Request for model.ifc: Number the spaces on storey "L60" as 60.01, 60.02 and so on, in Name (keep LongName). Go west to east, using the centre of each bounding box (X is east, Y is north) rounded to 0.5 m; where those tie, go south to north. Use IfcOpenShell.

First a look at what the model holds.

```python
import ifcopenshell
import ifcopenshell.util.element
import ifcopenshell.util.placement

model = ifcopenshell.open("model.ifc")
print(model.schema)
storey = next(s for s in model.by_type("IfcBuildingStorey") if s.Name == "L60")
spaces = [e for e in ifcopenshell.util.element.get_decomposition(storey) if e.is_a("IfcSpace")]
for e in sorted(spaces, key=lambda e: e.id()):
    origin = ifcopenshell.util.placement.get_local_placement(e.ObjectPlacement)[:3, 3]
    print(e.id(), e.Name, e.LongName, origin.round(2) + 0.0, sep=" | ")
```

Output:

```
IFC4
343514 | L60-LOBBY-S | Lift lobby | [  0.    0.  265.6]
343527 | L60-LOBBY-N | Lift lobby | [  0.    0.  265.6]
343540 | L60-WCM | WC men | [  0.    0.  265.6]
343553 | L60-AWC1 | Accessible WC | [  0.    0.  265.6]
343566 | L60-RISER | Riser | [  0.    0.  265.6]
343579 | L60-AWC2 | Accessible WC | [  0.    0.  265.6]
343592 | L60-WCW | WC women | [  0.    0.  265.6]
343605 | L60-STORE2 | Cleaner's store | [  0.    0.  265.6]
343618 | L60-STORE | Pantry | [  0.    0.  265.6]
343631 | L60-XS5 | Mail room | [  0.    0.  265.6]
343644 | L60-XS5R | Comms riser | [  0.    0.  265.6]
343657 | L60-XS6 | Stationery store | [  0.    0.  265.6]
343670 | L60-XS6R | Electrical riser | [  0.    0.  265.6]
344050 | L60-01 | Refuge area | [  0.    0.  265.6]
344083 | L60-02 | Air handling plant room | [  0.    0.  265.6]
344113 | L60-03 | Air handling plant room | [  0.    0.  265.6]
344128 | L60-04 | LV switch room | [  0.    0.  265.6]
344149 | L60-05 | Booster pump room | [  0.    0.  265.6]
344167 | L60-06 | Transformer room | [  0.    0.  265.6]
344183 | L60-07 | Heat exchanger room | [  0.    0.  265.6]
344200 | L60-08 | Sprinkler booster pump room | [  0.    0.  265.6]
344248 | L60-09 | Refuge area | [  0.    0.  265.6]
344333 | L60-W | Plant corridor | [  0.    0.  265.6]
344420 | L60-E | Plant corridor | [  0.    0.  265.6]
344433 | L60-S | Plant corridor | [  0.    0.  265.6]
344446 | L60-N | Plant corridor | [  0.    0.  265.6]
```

```python
import ifcopenshell
import ifcopenshell.geom
import ifcopenshell.util.element
import ifcopenshell.util.shape

model = ifcopenshell.open("model.ifc")
settings = ifcopenshell.geom.settings()
settings.set("use-world-coords", True)


def centre(element):
    shape = ifcopenshell.geom.create_shape(settings, element)
    return ifcopenshell.util.shape.get_bbox_centroid(shape.geometry)


storey = next(s for s in model.by_type("IfcBuildingStorey") if s.Name == "L60")
spaces = [e for e in ifcopenshell.util.element.get_decomposition(storey) if e.is_a("IfcSpace")]

# Insertion points can sit at a corner or the storey origin, so sort by the geometry (in metres).
centres = {e: centre(e) for e in spaces}
spaces.sort(key=lambda e: (round(centres[e][0] / 0.5), centres[e][1]))

for i, e in enumerate(spaces, start=1):
    number = f"60.{i:02d}"
    e.Name = number
    print(e.id(), number)

model.write("model-out.ifc")
```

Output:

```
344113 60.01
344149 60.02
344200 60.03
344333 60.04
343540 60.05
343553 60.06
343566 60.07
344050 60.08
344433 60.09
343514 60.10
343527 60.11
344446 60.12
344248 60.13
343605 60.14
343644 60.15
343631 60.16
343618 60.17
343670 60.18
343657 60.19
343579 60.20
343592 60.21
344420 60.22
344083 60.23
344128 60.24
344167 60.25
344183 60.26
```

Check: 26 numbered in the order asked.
